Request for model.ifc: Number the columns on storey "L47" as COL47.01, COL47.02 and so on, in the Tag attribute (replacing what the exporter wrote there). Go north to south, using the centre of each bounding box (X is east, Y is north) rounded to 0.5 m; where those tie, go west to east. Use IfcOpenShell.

First a look at what the model holds.

```python
import ifcopenshell
import ifcopenshell.util.element
import ifcopenshell.util.placement

model = ifcopenshell.open("model.ifc")
print(model.schema)
storey = next(s for s in model.by_type("IfcBuildingStorey") if s.Name == "L47")
columns = [e for e in ifcopenshell.util.element.get_decomposition(storey) if e.is_a("IfcColumn")]
for e in sorted(columns, key=lambda e: e.id()):
    origin = ifcopenshell.util.placement.get_local_placement(e.ObjectPlacement)[:3, 3]
    print(e.id(), e.Tag, e.Name, origin.round(2) + 0.0, sep=" | ")
```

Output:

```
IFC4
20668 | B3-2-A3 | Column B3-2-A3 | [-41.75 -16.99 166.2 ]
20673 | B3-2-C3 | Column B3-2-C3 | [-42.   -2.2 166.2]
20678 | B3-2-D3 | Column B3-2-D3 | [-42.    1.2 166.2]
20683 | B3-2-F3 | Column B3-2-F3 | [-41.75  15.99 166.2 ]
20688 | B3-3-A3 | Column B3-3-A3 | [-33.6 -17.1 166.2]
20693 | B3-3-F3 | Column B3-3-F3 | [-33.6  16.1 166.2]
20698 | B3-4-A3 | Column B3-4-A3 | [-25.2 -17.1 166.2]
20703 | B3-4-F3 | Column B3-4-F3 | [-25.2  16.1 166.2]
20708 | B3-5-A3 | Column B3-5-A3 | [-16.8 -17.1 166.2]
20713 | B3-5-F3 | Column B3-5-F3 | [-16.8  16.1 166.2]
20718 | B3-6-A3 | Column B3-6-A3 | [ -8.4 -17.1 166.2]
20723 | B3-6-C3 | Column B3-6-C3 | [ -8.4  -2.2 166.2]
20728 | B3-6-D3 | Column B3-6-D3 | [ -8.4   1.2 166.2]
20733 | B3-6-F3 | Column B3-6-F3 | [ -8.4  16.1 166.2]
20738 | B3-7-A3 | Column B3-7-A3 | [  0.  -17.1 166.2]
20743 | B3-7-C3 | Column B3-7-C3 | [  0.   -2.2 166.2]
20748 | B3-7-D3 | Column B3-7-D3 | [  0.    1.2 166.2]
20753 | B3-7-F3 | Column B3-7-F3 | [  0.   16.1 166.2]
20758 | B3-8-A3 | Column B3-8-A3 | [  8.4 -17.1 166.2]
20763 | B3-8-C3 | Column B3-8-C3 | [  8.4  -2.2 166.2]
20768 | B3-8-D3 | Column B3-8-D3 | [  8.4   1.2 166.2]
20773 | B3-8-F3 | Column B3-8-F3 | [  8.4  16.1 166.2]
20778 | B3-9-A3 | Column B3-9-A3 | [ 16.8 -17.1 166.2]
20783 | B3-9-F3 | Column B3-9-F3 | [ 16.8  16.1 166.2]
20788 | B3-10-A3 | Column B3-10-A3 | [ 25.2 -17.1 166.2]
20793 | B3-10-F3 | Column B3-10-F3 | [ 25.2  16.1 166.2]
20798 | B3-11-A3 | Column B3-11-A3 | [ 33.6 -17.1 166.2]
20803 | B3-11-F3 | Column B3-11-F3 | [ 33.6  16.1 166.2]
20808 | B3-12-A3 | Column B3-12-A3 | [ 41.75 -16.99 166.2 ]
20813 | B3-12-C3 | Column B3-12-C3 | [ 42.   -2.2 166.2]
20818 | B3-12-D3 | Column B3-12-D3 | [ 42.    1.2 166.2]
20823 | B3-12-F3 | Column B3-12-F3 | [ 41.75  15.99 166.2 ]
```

```python
import ifcopenshell
import ifcopenshell.geom
import ifcopenshell.util.element
import ifcopenshell.util.shape

model = ifcopenshell.open("model.ifc")
settings = ifcopenshell.geom.settings()
settings.set("use-world-coords", True)


def centre(element):
    shape = ifcopenshell.geom.create_shape(settings, element)
    return ifcopenshell.util.shape.get_bbox_centroid(shape.geometry)


storey = next(s for s in model.by_type("IfcBuildingStorey") if s.Name == "L47")
columns = [e for e in ifcopenshell.util.element.get_decomposition(storey) if e.is_a("IfcColumn")]

# Insertion points can sit at a corner or the storey origin, so sort by the geometry (in metres).
centres = {e: centre(e) for e in columns}
columns.sort(key=lambda e: (-round(centres[e][1] / 0.5), centres[e][0]))

for i, e in enumerate(columns, start=1):
    number = f"COL47.{i:02d}"
    e.Tag = number
    print(e.id(), number)

model.write("model-out.ifc")
```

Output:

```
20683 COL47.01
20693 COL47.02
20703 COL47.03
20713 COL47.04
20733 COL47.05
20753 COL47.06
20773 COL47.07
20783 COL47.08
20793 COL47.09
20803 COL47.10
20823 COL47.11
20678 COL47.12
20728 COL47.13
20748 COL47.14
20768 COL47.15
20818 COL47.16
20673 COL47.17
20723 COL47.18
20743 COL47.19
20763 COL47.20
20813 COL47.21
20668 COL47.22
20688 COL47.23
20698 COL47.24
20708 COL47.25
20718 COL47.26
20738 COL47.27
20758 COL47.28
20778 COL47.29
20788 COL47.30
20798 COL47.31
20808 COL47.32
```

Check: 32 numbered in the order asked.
